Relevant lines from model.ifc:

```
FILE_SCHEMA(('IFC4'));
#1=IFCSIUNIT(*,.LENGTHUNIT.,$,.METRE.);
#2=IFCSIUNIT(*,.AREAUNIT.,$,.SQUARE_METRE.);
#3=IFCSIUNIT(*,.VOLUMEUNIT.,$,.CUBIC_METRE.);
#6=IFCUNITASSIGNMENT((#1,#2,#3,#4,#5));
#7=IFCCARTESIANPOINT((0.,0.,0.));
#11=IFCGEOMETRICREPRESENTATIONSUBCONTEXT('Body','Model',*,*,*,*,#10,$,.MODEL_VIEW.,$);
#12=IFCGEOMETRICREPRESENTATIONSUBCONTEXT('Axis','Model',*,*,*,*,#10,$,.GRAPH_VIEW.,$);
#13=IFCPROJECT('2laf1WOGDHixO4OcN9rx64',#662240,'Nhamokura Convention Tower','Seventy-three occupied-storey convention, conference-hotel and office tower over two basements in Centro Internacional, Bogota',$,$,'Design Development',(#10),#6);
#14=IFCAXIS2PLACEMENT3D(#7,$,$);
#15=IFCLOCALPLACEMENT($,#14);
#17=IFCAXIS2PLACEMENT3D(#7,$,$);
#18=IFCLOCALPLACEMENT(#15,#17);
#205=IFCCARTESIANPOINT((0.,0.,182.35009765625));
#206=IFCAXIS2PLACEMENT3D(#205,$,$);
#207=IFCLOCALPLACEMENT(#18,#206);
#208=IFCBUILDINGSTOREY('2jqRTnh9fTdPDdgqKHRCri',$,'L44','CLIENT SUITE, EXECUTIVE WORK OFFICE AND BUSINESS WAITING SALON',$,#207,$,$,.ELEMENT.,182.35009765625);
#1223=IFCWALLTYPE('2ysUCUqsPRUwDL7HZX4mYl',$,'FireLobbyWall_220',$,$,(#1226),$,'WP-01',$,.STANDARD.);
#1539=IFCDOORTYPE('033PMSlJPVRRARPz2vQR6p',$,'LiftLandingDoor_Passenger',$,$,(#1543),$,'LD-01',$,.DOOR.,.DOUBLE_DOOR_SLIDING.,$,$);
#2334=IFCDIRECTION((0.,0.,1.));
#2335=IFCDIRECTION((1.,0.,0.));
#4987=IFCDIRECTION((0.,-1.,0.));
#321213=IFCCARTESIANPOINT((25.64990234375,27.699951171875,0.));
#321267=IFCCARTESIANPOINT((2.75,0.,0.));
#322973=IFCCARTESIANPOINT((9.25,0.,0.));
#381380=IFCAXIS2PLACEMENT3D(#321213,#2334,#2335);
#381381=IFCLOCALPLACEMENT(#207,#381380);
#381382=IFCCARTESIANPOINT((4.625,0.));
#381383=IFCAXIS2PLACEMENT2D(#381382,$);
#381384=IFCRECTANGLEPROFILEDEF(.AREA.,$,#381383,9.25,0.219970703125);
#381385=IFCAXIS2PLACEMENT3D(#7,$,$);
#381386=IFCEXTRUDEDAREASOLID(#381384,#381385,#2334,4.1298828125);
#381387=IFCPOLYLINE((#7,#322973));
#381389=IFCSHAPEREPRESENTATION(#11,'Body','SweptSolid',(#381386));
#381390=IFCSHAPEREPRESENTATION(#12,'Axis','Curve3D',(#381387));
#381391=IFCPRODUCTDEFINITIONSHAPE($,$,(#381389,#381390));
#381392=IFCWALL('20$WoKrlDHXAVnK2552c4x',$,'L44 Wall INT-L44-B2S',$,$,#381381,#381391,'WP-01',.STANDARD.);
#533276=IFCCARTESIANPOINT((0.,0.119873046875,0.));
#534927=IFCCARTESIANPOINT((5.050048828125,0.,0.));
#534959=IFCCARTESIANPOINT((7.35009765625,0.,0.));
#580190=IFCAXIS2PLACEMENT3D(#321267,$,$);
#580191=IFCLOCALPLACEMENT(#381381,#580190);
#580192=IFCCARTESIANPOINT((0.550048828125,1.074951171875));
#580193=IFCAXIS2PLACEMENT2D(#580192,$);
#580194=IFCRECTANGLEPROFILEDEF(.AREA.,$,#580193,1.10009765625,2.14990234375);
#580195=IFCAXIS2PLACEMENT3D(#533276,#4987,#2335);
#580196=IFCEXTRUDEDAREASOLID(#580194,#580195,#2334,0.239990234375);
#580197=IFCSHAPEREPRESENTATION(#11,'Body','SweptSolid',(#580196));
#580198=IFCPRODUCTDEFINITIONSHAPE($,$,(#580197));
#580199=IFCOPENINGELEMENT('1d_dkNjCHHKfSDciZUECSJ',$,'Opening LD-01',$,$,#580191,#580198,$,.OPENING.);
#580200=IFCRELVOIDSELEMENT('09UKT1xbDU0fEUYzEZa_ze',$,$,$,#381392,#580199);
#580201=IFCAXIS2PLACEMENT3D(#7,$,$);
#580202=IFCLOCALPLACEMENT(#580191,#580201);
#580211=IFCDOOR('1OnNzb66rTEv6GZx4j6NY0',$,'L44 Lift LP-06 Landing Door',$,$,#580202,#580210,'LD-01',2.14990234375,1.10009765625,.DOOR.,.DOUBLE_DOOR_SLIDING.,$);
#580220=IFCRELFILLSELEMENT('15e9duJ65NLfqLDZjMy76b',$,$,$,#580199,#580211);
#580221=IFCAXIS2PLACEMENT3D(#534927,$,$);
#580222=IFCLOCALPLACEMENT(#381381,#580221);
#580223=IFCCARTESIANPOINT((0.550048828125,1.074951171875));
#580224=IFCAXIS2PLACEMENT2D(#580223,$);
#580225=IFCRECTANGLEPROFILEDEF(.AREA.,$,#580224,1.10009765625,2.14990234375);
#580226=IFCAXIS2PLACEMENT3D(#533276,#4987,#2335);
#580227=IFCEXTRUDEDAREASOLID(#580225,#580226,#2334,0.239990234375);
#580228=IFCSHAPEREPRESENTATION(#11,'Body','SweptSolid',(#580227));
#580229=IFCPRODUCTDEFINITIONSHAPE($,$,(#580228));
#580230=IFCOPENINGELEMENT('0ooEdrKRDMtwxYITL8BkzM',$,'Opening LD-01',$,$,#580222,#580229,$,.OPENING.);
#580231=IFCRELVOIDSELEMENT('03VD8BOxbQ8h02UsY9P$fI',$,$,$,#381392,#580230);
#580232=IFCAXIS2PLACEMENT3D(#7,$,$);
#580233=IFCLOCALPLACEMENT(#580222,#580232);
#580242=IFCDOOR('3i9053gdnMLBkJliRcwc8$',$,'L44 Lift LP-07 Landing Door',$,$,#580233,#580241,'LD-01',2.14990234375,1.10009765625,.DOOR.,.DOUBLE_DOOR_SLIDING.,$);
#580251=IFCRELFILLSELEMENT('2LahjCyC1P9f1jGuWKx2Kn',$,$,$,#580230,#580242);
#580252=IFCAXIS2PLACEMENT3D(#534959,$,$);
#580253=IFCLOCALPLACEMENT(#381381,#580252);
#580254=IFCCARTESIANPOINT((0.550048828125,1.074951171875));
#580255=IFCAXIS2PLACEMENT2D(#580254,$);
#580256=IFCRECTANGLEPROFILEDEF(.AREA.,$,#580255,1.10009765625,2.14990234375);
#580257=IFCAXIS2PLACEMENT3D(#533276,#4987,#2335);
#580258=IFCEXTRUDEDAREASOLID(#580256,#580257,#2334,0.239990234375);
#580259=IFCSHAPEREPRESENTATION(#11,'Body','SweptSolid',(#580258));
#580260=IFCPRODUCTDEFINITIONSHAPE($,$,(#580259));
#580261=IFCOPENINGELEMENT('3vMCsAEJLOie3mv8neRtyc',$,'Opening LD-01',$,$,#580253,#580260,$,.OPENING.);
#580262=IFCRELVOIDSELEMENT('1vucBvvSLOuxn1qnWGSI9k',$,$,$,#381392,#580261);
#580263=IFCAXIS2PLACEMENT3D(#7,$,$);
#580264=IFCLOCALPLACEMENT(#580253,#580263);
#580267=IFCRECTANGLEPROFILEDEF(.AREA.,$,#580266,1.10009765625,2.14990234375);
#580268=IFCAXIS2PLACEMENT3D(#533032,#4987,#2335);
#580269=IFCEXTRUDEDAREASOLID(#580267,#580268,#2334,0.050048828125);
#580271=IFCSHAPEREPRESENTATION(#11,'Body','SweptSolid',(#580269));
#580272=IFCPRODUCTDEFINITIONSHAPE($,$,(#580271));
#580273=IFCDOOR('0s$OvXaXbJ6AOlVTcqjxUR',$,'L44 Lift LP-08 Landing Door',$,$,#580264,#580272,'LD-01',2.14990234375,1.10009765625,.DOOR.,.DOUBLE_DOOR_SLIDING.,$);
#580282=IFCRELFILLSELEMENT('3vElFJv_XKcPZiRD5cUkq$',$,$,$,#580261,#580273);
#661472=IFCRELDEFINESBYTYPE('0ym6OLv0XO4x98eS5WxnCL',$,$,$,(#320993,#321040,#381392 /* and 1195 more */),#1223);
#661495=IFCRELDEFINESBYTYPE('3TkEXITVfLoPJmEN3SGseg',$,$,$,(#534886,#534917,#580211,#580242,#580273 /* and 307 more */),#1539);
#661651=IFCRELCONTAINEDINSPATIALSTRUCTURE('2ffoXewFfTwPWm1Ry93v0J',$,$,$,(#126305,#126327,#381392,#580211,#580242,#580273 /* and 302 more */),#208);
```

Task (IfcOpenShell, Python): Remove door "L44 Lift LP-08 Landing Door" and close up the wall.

```python
import ifcopenshell
import ifcopenshell.api.feature
import ifcopenshell.api.root
import ifcopenshell.geom
import ifcopenshell.util.shape

model = ifcopenshell.open("model.ifc")
settings = ifcopenshell.geom.settings()


def volume(element):
    """Net volume in cubic metres, openings subtracted."""
    shape = ifcopenshell.geom.create_shape(settings, element)
    return ifcopenshell.util.shape.get_volume(shape.geometry)


door = model.by_guid("0s$OvXaXbJ6AOlVTcqjxUR")
opening = door.FillsVoids[0].RelatingOpeningElement
wall = opening.VoidsElements[0].RelatingBuildingElement
before = volume(wall)

ifcopenshell.api.root.remove_product(model, product=door)
ifcopenshell.api.feature.remove_feature(model, feature=opening)

after = volume(wall)

print(f"wall volume {before:.3f} -> {after:.3f} m3")

model.write("model_updated.ifc")
```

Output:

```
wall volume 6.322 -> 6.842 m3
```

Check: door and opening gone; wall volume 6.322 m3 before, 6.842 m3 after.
